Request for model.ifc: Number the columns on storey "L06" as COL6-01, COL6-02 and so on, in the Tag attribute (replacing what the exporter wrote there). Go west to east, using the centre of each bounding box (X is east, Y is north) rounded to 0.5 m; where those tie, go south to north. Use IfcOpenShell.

First a look at what the model holds.

```python
import ifcopenshell
import ifcopenshell.util.element
import ifcopenshell.util.placement

model = ifcopenshell.open("model.ifc")
print(model.schema)
storey = next(s for s in model.by_type("IfcBuildingStorey") if s.Name == "L06")
columns = [e for e in ifcopenshell.util.element.get_decomposition(storey) if e.is_a("IfcColumn")]
for e in sorted(columns, key=lambda e: e.id()):
    origin = ifcopenshell.util.placement.get_local_placement(e.ObjectPlacement)[:3, 3]
    print(e.id(), e.Tag, e.Name, origin.round(2) + 0.0, sep=" | ")
```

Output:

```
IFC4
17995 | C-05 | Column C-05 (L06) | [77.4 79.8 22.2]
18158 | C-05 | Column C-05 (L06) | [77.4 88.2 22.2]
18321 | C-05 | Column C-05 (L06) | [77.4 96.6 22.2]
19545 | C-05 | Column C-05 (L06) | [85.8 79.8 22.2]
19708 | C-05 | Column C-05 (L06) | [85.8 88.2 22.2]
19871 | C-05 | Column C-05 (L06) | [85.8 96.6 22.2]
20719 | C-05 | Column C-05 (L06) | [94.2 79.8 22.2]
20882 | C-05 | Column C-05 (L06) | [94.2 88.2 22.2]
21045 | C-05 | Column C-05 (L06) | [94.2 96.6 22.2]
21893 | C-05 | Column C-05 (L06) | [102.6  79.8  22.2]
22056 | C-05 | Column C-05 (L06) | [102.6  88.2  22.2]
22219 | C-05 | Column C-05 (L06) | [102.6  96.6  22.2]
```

```python
import ifcopenshell
import ifcopenshell.geom
import ifcopenshell.util.element
import ifcopenshell.util.shape

model = ifcopenshell.open("model.ifc")
settings = ifcopenshell.geom.settings()
settings.set("use-world-coords", True)


def centre(element):
    shape = ifcopenshell.geom.create_shape(settings, element)
    return ifcopenshell.util.shape.get_bbox_centroid(shape.geometry)


storey = next(s for s in model.by_type("IfcBuildingStorey") if s.Name == "L06")
columns = [e for e in ifcopenshell.util.element.get_decomposition(storey) if e.is_a("IfcColumn")]

# Insertion points can sit at a corner or the storey origin, so sort by the geometry (in metres).
centres = {e: centre(e) for e in columns}
columns.sort(key=lambda e: (round(centres[e][0] / 0.5), centres[e][1]))

for i, e in enumerate(columns, start=1):
    number = f"COL6-{i:02d}"
    e.Tag = number
    print(e.id(), number)

model.write("model_edited.ifc")
```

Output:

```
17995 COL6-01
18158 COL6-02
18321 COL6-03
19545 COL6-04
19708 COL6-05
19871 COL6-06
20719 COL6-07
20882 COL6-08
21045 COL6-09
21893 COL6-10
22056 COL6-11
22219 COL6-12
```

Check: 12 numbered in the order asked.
